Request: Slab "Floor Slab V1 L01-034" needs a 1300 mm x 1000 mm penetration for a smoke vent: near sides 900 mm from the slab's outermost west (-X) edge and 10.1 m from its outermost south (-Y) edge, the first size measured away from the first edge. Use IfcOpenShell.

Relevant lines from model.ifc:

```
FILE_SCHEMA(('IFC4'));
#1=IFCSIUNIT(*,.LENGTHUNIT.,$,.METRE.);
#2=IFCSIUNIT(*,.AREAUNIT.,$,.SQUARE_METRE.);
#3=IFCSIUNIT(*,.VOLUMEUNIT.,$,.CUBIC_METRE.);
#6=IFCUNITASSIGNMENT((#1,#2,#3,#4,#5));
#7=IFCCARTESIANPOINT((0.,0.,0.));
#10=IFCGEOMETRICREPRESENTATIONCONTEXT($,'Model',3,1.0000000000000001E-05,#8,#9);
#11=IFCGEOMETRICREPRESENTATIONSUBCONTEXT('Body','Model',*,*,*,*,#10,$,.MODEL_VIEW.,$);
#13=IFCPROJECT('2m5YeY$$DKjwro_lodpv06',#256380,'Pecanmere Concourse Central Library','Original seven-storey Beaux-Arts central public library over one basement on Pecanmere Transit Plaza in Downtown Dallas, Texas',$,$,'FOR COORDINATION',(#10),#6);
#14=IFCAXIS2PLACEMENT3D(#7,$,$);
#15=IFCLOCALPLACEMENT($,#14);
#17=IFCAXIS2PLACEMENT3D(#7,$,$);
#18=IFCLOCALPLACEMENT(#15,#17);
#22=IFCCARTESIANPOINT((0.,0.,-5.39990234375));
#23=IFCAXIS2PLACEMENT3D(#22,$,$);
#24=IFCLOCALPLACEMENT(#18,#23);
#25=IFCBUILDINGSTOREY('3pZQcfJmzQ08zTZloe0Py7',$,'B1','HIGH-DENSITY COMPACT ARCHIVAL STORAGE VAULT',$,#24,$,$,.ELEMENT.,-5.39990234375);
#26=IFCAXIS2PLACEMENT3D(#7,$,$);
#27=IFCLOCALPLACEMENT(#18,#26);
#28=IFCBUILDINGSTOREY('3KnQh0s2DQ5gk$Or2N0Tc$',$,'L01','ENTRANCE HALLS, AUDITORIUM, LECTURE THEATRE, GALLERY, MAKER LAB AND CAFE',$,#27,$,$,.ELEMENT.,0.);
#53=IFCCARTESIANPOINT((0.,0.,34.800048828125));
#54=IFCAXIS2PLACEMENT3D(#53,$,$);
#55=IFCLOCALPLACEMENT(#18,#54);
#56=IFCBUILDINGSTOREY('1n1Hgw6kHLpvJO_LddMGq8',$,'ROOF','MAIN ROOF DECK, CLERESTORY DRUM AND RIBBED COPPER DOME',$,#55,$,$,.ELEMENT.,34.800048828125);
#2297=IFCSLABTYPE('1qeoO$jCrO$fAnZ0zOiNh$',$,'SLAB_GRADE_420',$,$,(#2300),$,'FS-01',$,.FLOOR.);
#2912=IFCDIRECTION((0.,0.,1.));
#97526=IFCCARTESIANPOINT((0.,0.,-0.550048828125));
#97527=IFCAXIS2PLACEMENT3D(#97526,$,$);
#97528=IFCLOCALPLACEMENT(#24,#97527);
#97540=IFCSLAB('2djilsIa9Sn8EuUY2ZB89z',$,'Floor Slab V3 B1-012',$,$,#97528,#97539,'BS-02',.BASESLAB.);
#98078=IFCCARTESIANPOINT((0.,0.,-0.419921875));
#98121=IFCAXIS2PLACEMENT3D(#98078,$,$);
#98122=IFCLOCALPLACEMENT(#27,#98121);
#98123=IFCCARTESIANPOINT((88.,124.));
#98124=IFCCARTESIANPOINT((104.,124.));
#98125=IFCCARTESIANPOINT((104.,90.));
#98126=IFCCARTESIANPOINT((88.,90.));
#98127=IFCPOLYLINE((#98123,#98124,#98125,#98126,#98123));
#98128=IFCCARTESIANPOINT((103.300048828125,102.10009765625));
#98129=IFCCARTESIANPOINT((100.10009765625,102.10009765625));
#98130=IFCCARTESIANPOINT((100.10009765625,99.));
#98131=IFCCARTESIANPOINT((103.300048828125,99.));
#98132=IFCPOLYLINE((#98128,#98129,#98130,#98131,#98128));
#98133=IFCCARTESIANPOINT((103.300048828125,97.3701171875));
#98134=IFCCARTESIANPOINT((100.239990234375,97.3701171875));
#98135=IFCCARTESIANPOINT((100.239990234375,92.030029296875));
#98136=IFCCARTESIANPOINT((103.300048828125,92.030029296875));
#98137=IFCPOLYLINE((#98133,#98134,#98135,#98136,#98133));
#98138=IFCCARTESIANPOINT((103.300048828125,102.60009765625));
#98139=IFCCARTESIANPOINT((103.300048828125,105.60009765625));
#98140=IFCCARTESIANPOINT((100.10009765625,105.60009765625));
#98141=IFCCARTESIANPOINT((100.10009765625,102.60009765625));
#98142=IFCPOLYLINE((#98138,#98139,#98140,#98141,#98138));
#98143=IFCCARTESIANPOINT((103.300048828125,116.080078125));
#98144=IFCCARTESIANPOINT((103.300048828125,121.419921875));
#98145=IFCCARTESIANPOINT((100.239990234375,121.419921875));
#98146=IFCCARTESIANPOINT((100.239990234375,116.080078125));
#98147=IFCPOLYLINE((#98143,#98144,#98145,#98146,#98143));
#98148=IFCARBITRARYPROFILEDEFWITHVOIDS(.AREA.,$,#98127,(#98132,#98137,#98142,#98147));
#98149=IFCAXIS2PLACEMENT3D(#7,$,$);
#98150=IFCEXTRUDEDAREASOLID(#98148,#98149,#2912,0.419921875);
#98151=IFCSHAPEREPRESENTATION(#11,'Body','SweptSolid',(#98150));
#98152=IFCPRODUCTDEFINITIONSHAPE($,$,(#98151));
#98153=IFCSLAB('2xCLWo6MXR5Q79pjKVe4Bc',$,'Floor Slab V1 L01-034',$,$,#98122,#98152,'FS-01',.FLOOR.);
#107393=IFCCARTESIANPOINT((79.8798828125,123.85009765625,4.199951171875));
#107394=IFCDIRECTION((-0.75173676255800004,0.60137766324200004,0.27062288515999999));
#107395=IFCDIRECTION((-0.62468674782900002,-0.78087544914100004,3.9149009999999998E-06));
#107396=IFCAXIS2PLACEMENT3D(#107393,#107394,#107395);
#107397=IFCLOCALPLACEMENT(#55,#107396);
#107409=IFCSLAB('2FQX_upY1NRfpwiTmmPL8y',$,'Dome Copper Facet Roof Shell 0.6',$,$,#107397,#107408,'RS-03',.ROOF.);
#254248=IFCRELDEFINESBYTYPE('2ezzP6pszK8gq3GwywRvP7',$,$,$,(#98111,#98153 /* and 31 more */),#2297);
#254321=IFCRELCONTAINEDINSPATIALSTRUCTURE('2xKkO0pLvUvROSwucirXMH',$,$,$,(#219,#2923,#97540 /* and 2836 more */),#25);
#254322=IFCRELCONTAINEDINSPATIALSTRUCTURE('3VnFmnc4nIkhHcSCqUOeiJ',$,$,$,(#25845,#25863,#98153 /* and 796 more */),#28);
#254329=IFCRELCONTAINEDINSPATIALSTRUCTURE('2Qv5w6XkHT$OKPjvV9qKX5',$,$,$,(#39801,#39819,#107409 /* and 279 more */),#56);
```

```python
import numpy as np
import ifcopenshell
import ifcopenshell.api.feature
import ifcopenshell.api.geometry
import ifcopenshell.api.root
import ifcopenshell.geom
import ifcopenshell.util.placement
import ifcopenshell.util.representation
import ifcopenshell.util.shape
import ifcopenshell.util.unit

model = ifcopenshell.open("model.ifc")
unit_scale = ifcopenshell.util.unit.calculate_unit_scale(model)
settings = ifcopenshell.geom.settings()


def volume(element):
    """Net volume in cubic metres, openings subtracted."""
    shape = ifcopenshell.geom.create_shape(settings, element)
    return ifcopenshell.util.shape.get_volume(shape.geometry)


slab = model.by_guid("2xCLWo6MXR5Q79pjKVe4Bc")
before = volume(slab)

# Extent in the slab's own axes, in metres. The edges named are its -X and -Y sides.
slab_shape = ifcopenshell.geom.create_shape(settings, slab)
vertices = ifcopenshell.util.shape.get_vertices(slab_shape.geometry)
x_min, y_min, bottom = vertices.min(axis=0)
top = vertices[:, 2].max()

opening = ifcopenshell.api.root.create_entity(model, ifc_class="IfcOpeningElement", name="Smoke vent opening", predefined_type="OPENING")
context = ifcopenshell.util.representation.get_context(model, "Model", "Body", "MODEL_VIEW")
width, depth = 1.3, 1
outline = [(0.0, 0.0), (width, 0.0), (width, depth), (0.0, depth), (0.0, 0.0)]
# Overshoot both faces by 50 mm so the cut is clean.
shape = ifcopenshell.api.geometry.add_slab_representation(
    model, context=context, depth=top - bottom + 0.1, polyline=outline
)
ifcopenshell.api.geometry.assign_representation(model, product=opening, representation=shape)

matrix = ifcopenshell.util.placement.get_local_placement(slab.ObjectPlacement)
matrix[:, 3] = matrix @ np.append(np.array([x_min + 0.9, y_min + 10.1, bottom - 0.05]) / unit_scale, 1.0)
ifcopenshell.api.geometry.edit_object_placement(model, product=opening, matrix=matrix, is_si=False)
ifcopenshell.api.feature.add_feature(model, feature=opening, element=slab)

after = volume(slab)

print(f"slab volume {before:.3f} -> {after:.3f} m3")

model.write("model_updated.ifc")
```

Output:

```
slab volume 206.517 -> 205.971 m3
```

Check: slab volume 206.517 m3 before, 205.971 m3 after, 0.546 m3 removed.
